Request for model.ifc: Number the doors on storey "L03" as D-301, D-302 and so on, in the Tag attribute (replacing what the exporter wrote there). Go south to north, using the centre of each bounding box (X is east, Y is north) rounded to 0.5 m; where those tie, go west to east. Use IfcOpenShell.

First a look at what the model holds.

```python
import ifcopenshell
import ifcopenshell.util.element
import ifcopenshell.util.placement

model = ifcopenshell.open("model.ifc")
print(model.schema)
storey = next(s for s in model.by_type("IfcBuildingStorey") if s.Name == "L03")
doors = [e for e in ifcopenshell.util.element.get_decomposition(storey) if e.is_a("IfcDoor")]
for e in sorted(doors, key=lambda e: e.id()):
    origin = ifcopenshell.util.placement.get_local_placement(e.ObjectPlacement)[:3, 3]
    print(e.id(), e.Tag, e.Name, origin.round(2) + 0.0, sep=" | ")
```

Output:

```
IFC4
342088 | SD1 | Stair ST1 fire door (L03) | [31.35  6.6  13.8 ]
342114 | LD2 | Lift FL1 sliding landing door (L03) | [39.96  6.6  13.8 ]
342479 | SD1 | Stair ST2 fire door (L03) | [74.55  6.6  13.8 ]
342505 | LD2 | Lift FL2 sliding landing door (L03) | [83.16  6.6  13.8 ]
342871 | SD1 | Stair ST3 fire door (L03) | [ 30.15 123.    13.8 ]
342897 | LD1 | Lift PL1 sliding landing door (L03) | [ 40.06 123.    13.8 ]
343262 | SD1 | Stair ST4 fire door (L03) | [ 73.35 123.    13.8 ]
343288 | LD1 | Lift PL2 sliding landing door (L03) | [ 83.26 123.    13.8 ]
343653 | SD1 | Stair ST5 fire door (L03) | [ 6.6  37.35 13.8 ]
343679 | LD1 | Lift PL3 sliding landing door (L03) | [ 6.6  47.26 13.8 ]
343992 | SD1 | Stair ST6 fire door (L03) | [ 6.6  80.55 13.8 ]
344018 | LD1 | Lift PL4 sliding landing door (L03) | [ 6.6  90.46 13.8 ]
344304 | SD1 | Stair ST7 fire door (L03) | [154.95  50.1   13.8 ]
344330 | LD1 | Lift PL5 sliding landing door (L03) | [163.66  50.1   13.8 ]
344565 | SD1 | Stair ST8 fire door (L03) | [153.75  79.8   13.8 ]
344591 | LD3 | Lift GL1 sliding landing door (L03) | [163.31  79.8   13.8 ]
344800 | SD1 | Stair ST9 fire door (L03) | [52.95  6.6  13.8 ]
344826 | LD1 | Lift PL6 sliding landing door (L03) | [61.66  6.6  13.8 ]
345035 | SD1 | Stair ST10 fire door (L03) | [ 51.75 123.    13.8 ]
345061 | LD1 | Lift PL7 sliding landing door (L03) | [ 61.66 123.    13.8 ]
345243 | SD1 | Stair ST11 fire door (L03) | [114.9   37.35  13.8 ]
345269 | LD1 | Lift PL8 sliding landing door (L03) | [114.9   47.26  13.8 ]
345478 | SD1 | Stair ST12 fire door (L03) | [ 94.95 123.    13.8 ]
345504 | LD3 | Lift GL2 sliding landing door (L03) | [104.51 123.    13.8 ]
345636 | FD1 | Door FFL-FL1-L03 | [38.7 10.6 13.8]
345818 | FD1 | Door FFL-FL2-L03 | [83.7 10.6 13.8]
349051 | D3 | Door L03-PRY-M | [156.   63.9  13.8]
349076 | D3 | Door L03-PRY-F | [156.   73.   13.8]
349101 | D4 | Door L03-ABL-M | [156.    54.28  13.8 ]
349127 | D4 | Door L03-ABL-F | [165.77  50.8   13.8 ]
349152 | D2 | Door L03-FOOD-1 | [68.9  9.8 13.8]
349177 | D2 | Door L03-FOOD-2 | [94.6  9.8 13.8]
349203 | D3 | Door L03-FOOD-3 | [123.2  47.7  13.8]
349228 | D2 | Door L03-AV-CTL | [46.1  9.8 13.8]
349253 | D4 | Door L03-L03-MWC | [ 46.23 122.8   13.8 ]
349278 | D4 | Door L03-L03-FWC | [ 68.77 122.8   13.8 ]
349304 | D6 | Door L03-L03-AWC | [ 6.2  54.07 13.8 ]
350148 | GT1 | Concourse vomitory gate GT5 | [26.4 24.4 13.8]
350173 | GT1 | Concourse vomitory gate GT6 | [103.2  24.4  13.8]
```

```python
import ifcopenshell
import ifcopenshell.geom
import ifcopenshell.util.element
import ifcopenshell.util.shape

model = ifcopenshell.open("model.ifc")
settings = ifcopenshell.geom.settings()
settings.set("use-world-coords", True)


def centre(element):
    shape = ifcopenshell.geom.create_shape(settings, element)
    return ifcopenshell.util.shape.get_bbox_centroid(shape.geometry)


storey = next(s for s in model.by_type("IfcBuildingStorey") if s.Name == "L03")
doors = [e for e in ifcopenshell.util.element.get_decomposition(storey) if e.is_a("IfcDoor")]

# Insertion points can sit at a corner or the storey origin, so sort by the geometry (in metres).
centres = {e: centre(e) for e in doors}
doors.sort(key=lambda e: (round(centres[e][1] / 0.5), centres[e][0]))

for i, e in enumerate(doors, start=1):
    number = f"D-3{i:02d}"
    e.Tag = number
    print(e.id(), number)

model.write("model_rev.ifc")
```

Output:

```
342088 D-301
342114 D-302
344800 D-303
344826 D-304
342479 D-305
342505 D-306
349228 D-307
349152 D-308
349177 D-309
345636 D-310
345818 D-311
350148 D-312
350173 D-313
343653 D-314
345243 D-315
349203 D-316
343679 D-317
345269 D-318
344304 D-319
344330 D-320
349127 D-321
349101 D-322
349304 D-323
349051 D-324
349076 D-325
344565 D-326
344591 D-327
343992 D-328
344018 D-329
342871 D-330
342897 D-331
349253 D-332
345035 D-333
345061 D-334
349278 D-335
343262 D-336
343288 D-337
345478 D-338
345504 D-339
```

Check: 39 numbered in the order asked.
